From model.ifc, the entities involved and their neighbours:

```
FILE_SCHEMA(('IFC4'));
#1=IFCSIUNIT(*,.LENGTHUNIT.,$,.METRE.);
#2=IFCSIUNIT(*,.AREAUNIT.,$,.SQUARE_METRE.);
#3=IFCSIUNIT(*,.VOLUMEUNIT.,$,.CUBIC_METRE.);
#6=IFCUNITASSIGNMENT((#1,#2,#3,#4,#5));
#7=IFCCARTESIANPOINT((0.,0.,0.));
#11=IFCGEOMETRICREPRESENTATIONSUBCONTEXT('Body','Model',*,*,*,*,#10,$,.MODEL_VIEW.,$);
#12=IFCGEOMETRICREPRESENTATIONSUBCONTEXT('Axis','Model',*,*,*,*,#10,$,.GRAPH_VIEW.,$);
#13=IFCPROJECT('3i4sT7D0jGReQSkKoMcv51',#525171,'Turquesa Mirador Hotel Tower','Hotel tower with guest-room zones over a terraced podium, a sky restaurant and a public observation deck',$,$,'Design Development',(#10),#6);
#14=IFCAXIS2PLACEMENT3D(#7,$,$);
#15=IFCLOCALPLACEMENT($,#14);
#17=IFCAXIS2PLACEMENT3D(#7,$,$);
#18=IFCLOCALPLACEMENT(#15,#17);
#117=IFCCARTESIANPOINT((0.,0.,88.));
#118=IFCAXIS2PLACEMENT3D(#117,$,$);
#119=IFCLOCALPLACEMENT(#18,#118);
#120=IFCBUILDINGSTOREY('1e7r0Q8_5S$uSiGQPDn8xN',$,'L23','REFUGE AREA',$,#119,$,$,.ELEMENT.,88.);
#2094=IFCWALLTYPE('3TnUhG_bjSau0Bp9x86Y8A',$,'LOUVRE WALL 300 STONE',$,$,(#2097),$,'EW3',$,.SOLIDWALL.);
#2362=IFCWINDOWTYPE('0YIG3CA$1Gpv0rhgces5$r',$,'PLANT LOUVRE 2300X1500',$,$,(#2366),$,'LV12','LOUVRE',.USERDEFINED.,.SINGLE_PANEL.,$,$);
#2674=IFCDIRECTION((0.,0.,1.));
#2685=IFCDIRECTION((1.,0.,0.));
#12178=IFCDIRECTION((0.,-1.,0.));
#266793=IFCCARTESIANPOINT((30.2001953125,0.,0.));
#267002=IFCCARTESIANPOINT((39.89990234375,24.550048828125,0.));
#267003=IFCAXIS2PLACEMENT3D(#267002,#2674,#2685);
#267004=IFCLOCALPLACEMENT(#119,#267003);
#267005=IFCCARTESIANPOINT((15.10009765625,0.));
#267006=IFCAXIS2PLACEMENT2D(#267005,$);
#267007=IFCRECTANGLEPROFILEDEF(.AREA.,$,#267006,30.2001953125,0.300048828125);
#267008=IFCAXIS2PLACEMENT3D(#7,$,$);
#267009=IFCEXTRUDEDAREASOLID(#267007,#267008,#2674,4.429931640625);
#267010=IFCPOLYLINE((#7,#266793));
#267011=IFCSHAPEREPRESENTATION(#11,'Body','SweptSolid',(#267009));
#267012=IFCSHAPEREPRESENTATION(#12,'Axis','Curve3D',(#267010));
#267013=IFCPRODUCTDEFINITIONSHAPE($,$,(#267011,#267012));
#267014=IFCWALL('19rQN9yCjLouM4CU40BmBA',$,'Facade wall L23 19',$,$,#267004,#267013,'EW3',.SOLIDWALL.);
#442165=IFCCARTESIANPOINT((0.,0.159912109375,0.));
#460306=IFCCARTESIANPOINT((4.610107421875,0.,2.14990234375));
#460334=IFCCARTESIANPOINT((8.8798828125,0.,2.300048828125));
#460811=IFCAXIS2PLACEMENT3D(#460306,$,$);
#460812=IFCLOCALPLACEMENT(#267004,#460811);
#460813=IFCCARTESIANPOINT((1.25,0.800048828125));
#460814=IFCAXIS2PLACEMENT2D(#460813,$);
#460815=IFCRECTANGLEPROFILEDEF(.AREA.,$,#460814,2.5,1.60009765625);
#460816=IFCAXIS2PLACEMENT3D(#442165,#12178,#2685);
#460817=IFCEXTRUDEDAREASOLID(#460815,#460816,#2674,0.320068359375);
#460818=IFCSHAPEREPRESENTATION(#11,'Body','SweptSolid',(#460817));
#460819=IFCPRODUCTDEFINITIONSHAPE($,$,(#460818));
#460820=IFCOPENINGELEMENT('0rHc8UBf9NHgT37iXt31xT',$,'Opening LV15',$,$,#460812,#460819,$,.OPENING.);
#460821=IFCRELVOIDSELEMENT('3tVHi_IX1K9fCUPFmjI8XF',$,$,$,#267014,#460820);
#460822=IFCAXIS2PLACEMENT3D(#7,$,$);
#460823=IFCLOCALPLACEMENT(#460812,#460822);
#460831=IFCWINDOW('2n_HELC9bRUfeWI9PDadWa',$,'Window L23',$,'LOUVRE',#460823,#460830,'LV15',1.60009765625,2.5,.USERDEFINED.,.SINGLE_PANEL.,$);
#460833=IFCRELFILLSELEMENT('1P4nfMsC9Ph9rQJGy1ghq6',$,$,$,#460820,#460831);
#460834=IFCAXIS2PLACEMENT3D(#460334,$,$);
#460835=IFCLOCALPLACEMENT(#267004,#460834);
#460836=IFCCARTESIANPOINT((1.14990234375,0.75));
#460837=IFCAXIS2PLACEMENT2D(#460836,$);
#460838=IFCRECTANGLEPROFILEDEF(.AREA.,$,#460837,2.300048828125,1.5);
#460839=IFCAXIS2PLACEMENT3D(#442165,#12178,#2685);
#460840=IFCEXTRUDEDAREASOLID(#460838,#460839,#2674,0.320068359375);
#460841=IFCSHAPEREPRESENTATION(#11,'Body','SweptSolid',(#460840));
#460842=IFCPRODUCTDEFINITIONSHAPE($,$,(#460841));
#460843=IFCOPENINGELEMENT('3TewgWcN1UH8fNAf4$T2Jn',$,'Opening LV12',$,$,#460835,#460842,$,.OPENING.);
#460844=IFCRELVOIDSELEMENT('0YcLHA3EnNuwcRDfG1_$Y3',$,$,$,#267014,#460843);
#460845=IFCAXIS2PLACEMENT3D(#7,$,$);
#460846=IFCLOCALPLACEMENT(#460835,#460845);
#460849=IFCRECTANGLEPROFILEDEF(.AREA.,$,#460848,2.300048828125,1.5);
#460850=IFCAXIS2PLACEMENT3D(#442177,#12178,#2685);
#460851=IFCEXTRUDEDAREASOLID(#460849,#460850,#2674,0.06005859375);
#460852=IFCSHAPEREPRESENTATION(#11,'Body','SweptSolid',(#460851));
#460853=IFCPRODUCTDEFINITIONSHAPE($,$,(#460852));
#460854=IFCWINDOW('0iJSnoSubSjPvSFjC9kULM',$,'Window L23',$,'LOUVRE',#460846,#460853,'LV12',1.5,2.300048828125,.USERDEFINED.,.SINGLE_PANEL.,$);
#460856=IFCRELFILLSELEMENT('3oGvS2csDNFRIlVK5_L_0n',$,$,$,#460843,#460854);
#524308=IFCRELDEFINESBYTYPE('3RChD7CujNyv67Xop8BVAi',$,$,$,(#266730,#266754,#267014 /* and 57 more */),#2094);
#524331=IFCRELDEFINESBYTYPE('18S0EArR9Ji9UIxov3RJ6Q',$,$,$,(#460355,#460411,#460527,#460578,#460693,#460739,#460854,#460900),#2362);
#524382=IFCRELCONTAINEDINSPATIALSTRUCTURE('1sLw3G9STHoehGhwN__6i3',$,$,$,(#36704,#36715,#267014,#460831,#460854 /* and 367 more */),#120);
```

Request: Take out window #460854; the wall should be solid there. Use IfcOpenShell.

```python
import ifcopenshell
import ifcopenshell.api.feature
import ifcopenshell.api.root
import ifcopenshell.geom
import ifcopenshell.util.shape

model = ifcopenshell.open("model.ifc")
settings = ifcopenshell.geom.settings()


def volume(element):
    """Net volume in cubic metres, openings subtracted."""
    shape = ifcopenshell.geom.create_shape(settings, element)
    return ifcopenshell.util.shape.get_volume(shape.geometry)


window = model.by_id(460854)
opening = window.FillsVoids[0].RelatingOpeningElement
wall = opening.VoidsElements[0].RelatingBuildingElement
before = volume(wall)

ifcopenshell.api.root.remove_product(model, product=window)
ifcopenshell.api.feature.remove_feature(model, feature=opening)

after = volume(wall)

print(f"wall volume {before:.3f} -> {after:.3f} m3")

model.write("model-out.ifc")
```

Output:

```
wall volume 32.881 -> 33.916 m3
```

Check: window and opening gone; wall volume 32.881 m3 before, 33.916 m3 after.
